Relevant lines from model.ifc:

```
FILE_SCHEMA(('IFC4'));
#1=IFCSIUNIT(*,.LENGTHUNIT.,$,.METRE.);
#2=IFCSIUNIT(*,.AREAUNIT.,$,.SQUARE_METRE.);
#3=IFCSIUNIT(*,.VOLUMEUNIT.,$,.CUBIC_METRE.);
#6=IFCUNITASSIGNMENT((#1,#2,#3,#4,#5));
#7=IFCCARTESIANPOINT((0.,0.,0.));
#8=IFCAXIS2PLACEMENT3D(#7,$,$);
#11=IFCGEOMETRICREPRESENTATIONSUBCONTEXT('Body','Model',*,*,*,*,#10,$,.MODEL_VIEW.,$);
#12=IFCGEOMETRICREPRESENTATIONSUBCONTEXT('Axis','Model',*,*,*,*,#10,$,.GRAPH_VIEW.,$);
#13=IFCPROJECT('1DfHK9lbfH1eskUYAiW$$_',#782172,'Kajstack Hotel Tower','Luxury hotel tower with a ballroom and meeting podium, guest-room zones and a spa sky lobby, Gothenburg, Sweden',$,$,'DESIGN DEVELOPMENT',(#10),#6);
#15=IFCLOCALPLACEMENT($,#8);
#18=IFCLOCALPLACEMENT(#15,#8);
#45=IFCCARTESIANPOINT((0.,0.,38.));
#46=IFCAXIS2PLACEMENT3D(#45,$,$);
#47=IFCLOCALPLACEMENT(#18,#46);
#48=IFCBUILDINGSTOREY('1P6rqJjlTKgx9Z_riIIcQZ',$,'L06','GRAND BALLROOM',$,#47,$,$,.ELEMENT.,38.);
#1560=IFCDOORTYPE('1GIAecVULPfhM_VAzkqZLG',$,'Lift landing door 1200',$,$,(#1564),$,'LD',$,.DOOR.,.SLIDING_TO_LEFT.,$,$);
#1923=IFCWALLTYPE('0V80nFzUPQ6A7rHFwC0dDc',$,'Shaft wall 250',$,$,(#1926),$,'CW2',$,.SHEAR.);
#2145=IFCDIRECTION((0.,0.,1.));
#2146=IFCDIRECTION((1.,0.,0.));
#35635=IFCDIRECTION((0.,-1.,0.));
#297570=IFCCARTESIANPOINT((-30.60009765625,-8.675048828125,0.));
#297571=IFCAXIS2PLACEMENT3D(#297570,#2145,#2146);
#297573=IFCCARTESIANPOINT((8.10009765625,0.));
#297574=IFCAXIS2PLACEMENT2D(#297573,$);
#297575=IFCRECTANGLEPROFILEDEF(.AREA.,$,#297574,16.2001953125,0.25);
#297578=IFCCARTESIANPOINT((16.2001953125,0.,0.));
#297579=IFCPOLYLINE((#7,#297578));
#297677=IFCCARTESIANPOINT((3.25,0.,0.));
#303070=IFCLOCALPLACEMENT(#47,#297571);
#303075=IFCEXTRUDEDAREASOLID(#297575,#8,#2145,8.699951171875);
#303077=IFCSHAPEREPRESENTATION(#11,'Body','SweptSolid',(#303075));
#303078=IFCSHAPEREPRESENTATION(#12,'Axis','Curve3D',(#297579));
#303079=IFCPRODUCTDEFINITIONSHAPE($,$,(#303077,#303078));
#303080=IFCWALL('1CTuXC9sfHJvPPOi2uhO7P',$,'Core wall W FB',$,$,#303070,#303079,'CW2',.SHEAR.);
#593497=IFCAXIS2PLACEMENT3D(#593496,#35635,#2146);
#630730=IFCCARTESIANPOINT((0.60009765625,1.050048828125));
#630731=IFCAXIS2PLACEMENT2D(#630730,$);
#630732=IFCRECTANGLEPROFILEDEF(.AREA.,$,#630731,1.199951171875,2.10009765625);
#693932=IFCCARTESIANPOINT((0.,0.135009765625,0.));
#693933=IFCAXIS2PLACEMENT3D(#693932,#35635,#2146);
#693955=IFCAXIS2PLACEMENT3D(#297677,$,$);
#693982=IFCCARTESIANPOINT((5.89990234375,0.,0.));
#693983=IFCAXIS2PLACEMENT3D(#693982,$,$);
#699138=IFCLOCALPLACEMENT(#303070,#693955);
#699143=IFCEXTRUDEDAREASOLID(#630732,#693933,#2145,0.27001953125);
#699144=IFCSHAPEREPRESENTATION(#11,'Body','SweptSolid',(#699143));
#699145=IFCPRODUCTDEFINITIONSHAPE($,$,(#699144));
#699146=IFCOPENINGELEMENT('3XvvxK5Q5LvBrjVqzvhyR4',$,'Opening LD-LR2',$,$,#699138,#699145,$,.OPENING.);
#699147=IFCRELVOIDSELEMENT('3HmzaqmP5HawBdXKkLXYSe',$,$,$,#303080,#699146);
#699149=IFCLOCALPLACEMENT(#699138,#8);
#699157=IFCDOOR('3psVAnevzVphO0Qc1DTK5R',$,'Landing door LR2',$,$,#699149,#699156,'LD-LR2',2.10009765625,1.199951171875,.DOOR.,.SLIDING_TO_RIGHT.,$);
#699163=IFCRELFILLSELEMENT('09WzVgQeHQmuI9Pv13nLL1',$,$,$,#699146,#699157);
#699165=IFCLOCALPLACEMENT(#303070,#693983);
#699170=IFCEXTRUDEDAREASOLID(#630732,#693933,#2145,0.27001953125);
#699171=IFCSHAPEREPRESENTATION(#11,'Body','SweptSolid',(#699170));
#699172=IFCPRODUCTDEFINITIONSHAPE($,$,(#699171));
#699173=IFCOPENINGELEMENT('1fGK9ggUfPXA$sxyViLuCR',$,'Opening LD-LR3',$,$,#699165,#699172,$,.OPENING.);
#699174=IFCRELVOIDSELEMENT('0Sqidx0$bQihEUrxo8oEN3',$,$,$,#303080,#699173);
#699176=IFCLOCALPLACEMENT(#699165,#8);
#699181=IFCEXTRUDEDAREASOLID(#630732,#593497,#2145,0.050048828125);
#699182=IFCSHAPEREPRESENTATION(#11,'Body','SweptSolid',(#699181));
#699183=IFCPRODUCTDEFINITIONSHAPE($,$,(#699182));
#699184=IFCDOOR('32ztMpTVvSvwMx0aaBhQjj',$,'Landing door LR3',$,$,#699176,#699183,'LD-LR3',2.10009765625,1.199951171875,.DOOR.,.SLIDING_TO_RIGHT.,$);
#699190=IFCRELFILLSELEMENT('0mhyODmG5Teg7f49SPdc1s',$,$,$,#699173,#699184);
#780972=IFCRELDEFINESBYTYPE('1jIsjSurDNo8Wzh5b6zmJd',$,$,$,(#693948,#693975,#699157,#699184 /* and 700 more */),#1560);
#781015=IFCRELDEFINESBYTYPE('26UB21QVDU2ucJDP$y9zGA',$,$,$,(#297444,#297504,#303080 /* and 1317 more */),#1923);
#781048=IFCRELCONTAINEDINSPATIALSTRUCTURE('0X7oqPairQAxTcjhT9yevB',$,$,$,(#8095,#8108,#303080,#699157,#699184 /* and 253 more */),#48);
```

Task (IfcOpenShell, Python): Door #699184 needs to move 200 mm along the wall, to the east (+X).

```python
import ifcopenshell
import ifcopenshell.api.geometry
import ifcopenshell.util.placement
import ifcopenshell.util.unit

model = ifcopenshell.open("model.ifc")
unit_scale = ifcopenshell.util.unit.calculate_unit_scale(model)

door = model.by_guid("32ztMpTVvSvwMx0aaBhQjj")
opening = door.FillsVoids[0].RelatingOpeningElement
wall = opening.VoidsElements[0].RelatingBuildingElement

wall_matrix = ifcopenshell.util.placement.get_local_placement(wall.ObjectPlacement)
shift = wall_matrix[:3, 0] * 0.2 / unit_scale
before = ifcopenshell.util.placement.get_local_placement(door.ObjectPlacement)[:3, 3].copy()

# The door is placed relative to its opening, so it follows when the opening moves.
matrix = ifcopenshell.util.placement.get_local_placement(opening.ObjectPlacement)
matrix[:3, 3] += shift
ifcopenshell.api.geometry.edit_object_placement(
    model, product=opening, matrix=matrix, is_si=False, should_transform_children=True
)

after = ifcopenshell.util.placement.get_local_placement(door.ObjectPlacement)[:3, 3]
print("door moved by", (after - before).round(3) + 0.0)

model.write("model_edited.ifc")
```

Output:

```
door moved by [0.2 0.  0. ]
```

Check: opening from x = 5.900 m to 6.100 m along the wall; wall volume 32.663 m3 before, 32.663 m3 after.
